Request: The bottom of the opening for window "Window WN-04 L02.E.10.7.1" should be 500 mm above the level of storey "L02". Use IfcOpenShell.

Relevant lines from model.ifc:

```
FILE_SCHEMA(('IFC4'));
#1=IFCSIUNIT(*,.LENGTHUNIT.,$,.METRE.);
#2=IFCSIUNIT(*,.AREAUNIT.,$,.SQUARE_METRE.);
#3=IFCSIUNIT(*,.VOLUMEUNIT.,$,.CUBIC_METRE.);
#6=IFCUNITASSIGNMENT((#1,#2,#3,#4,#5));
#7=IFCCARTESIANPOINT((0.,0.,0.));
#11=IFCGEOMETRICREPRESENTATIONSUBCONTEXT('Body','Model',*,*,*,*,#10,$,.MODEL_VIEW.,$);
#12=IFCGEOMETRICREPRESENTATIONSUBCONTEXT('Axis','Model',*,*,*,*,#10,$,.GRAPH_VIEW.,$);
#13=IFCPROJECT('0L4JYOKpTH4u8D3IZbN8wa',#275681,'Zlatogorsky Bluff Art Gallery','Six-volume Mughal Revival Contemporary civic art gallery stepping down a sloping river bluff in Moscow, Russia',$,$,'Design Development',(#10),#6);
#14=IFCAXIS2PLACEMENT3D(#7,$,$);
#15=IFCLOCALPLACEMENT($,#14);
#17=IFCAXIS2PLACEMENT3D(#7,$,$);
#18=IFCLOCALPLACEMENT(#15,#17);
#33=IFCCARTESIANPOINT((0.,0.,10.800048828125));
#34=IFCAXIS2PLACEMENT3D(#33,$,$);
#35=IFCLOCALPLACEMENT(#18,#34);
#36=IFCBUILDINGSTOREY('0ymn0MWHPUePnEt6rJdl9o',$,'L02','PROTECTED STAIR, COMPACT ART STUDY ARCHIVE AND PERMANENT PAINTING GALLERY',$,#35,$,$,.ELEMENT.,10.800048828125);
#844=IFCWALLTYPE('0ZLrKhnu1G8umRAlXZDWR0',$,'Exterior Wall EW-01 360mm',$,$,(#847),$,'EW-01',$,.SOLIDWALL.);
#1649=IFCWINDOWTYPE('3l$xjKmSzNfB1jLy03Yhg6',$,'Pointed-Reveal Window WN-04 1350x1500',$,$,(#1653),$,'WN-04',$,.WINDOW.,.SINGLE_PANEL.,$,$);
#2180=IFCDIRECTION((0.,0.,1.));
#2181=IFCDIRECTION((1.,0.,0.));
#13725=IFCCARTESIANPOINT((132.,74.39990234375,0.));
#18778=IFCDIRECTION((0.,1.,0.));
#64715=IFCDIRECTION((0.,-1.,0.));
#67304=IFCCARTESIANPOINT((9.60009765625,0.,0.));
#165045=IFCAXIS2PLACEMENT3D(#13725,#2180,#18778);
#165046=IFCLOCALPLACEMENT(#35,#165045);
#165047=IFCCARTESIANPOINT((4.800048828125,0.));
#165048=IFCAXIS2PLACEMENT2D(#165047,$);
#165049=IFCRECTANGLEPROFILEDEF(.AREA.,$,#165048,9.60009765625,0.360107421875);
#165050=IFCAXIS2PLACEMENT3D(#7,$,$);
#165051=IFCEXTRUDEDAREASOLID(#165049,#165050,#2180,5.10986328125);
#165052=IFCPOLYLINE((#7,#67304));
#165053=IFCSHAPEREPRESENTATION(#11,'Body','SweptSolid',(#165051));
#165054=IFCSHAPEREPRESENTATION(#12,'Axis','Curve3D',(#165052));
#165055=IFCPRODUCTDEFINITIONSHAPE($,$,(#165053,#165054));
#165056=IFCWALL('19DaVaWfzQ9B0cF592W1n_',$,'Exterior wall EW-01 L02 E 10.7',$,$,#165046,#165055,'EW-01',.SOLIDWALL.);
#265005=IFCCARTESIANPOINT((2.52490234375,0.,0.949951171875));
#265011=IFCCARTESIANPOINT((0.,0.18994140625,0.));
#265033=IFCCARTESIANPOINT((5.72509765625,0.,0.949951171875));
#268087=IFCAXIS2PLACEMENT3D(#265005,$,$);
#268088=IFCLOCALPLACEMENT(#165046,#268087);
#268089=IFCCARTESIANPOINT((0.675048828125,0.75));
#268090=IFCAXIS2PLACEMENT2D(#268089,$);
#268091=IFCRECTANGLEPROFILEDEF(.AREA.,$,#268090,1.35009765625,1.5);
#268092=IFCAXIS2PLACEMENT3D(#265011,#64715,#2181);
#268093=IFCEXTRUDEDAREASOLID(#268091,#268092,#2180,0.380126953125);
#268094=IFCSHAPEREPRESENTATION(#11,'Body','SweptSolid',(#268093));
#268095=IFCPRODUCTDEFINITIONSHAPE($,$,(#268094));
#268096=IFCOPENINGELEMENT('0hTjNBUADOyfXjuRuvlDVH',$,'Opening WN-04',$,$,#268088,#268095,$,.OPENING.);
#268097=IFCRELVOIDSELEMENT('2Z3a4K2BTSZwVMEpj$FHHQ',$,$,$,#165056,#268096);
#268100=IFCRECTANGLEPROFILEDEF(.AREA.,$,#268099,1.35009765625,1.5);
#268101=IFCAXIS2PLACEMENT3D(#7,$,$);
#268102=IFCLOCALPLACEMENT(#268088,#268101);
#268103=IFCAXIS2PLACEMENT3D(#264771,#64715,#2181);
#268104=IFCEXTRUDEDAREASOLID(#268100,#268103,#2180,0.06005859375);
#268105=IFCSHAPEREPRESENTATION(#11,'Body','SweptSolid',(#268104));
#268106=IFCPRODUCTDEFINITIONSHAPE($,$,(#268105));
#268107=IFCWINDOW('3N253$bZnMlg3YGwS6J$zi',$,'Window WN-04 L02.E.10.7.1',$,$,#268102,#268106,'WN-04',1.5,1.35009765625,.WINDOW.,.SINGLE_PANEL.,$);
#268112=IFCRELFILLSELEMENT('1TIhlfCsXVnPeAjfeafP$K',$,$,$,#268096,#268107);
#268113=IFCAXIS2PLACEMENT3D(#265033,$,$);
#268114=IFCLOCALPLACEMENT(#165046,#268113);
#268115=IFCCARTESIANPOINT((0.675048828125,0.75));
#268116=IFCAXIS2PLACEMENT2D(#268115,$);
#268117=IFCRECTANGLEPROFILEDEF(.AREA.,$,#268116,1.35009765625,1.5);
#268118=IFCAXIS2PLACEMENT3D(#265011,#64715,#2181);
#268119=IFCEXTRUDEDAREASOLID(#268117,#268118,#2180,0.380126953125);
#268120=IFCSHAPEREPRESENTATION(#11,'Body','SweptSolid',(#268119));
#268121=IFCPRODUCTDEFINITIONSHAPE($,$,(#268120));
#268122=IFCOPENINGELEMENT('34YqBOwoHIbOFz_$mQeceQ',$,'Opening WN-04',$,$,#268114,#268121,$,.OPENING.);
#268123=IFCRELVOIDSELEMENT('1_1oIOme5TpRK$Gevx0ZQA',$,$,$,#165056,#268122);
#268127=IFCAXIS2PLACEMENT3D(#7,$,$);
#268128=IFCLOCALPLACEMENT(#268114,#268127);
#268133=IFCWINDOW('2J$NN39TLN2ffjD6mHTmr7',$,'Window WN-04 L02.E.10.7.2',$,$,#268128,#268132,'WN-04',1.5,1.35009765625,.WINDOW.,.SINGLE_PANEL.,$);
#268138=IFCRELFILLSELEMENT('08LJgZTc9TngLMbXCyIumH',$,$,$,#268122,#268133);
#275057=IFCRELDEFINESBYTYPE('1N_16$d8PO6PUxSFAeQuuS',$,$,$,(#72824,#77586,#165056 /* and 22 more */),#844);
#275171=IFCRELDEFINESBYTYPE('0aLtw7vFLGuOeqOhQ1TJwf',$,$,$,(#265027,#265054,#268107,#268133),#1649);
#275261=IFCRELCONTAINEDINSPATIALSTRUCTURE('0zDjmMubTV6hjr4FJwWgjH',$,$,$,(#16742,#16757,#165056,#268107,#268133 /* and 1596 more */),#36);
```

```python
import numpy as np
import ifcopenshell
import ifcopenshell.api.geometry
import ifcopenshell.geom
import ifcopenshell.util.element
import ifcopenshell.util.placement
import ifcopenshell.util.shape
import ifcopenshell.util.unit

model = ifcopenshell.open("model.ifc")
unit_scale = ifcopenshell.util.unit.calculate_unit_scale(model)

window = model.by_guid("3N253$bZnMlg3YGwS6J$zi")
opening = window.FillsVoids[0].RelatingOpeningElement
storey = ifcopenshell.util.element.get_container(window, ifc_class="IfcBuildingStorey")
level = ifcopenshell.util.placement.get_local_placement(storey.ObjectPlacement)[2, 3]

# The opening's origin need not be at the sill, so measure its lowest point.
shape = ifcopenshell.geom.create_shape(ifcopenshell.geom.settings(), opening)
bottom = ifcopenshell.util.shape.get_shape_bottom_elevation(shape, shape.geometry) / unit_scale
dz = level + 0.5 - bottom

shift = np.array([0.0, 0.0, dz])
# The window is placed relative to its opening, so it follows when the opening moves.
matrix = ifcopenshell.util.placement.get_local_placement(opening.ObjectPlacement)
matrix[:3, 3] += shift
ifcopenshell.api.geometry.edit_object_placement(
    model, product=opening, matrix=matrix, is_si=False, should_transform_children=True
)

print(f"moved by {dz * unit_scale:+.3f} m")

model.write("model_v2.ifc")
```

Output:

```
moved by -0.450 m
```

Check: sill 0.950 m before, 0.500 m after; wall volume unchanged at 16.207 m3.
